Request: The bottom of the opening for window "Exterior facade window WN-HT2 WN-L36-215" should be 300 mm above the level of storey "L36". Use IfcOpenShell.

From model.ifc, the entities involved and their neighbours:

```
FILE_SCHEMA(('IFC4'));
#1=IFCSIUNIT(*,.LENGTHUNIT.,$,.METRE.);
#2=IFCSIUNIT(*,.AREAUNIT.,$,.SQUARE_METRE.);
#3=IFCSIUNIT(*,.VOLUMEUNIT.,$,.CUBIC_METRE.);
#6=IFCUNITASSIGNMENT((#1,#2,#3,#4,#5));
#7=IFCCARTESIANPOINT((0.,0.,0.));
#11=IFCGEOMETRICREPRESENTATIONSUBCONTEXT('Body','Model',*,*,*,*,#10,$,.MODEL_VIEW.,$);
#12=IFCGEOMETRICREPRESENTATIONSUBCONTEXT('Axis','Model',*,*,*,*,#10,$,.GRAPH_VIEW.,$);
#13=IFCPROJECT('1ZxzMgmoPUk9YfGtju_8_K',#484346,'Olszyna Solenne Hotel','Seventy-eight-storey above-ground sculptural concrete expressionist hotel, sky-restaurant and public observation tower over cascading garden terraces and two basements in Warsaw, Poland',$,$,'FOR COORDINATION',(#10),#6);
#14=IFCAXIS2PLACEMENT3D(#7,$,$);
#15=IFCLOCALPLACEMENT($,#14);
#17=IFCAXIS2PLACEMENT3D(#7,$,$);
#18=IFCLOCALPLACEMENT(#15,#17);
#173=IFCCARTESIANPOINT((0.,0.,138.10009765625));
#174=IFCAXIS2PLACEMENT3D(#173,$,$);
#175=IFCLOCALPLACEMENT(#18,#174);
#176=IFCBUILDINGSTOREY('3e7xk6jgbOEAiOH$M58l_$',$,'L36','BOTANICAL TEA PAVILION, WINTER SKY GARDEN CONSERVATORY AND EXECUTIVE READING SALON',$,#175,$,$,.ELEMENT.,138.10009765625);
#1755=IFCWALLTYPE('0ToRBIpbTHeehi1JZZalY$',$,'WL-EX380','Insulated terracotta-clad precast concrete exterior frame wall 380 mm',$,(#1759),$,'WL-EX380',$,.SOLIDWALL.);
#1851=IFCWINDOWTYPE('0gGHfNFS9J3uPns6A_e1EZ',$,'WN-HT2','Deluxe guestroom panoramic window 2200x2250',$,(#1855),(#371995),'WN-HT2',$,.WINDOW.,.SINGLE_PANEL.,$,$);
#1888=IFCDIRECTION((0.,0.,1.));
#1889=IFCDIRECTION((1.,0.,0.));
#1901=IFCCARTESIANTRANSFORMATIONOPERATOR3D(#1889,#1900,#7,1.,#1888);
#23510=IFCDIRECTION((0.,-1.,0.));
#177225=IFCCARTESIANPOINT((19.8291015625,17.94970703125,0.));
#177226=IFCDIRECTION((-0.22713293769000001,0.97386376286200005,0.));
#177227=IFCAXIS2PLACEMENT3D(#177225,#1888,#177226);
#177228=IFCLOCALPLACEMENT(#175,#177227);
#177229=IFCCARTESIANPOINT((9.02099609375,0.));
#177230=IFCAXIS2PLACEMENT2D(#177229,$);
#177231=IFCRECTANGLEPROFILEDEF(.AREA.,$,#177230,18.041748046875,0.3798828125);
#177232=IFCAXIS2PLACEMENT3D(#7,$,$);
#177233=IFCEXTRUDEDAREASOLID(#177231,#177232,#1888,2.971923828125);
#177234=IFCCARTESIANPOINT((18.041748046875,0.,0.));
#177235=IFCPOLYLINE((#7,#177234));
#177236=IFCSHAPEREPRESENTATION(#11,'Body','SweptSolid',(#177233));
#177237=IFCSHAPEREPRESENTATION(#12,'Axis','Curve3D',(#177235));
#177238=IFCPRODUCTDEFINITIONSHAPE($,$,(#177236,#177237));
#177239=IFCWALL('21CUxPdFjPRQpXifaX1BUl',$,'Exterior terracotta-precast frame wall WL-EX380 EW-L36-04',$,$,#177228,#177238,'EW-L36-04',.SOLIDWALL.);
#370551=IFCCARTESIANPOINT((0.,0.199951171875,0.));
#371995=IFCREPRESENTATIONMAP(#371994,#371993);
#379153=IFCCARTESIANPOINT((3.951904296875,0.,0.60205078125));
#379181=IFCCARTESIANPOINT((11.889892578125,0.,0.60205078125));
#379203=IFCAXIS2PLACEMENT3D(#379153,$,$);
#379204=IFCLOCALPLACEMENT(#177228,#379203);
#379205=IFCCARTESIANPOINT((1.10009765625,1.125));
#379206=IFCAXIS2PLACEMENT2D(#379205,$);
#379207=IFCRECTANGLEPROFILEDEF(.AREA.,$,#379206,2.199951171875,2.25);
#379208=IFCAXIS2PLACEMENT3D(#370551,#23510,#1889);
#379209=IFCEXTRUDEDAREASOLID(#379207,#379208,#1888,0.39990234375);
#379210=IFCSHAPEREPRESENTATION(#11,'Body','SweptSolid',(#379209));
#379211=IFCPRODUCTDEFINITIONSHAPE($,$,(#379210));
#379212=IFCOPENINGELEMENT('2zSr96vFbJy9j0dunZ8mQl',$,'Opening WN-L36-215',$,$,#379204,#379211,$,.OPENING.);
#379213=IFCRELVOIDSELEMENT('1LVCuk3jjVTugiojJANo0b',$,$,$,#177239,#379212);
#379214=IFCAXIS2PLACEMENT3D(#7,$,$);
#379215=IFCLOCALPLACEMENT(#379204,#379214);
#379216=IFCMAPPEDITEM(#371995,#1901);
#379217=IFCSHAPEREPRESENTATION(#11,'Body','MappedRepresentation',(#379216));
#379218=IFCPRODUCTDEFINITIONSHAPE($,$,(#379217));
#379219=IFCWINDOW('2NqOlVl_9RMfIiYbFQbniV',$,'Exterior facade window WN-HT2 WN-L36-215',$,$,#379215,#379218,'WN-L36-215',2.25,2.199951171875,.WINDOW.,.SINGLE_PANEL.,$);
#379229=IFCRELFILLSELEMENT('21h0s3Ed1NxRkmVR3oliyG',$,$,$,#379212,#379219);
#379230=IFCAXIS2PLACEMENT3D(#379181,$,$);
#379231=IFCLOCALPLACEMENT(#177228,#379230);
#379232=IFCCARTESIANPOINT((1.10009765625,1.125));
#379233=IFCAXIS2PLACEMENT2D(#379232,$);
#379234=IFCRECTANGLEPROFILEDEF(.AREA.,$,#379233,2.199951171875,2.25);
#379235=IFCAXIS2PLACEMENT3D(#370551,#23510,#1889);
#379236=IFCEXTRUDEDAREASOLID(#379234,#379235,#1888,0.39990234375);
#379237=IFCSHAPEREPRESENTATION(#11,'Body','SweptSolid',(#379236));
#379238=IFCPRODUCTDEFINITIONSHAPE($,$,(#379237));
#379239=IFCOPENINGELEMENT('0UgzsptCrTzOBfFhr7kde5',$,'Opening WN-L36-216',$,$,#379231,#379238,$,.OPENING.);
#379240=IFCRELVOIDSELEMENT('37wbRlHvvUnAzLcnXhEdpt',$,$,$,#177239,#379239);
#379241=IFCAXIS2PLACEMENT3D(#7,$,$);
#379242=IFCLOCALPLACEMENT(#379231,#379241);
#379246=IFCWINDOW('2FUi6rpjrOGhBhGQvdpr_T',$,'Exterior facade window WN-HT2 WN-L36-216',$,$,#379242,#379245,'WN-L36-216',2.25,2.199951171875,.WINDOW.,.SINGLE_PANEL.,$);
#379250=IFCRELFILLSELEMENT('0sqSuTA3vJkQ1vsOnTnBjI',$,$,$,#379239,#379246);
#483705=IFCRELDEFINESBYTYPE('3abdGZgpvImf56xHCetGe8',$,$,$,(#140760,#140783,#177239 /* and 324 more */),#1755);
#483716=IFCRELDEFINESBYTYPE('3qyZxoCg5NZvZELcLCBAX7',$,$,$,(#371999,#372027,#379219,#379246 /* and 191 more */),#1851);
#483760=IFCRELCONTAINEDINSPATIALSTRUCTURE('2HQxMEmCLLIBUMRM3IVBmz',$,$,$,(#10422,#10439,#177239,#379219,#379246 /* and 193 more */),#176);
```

```python
import numpy as np
import ifcopenshell
import ifcopenshell.api.geometry
import ifcopenshell.geom
import ifcopenshell.util.element
import ifcopenshell.util.placement
import ifcopenshell.util.shape
import ifcopenshell.util.unit

model = ifcopenshell.open("model.ifc")
unit_scale = ifcopenshell.util.unit.calculate_unit_scale(model)

window = model.by_guid("2NqOlVl_9RMfIiYbFQbniV")
opening = window.FillsVoids[0].RelatingOpeningElement
storey = ifcopenshell.util.element.get_container(window, ifc_class="IfcBuildingStorey")
level = ifcopenshell.util.placement.get_local_placement(storey.ObjectPlacement)[2, 3]

# The opening's origin need not be at the sill, so measure its lowest point.
shape = ifcopenshell.geom.create_shape(ifcopenshell.geom.settings(), opening)
bottom = ifcopenshell.util.shape.get_shape_bottom_elevation(shape, shape.geometry) / unit_scale
dz = level + 0.3 - bottom

shift = np.array([0.0, 0.0, dz])
# The window is placed relative to its opening, so it follows when the opening moves.
matrix = ifcopenshell.util.placement.get_local_placement(opening.ObjectPlacement)
matrix[:3, 3] += shift
ifcopenshell.api.geometry.edit_object_placement(
    model, product=opening, matrix=matrix, is_si=False, should_transform_children=True
)

print(f"moved by {dz * unit_scale:+.3f} m")

model.write("model_v2.ifc")
```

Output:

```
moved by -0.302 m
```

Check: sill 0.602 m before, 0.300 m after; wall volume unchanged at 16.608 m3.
